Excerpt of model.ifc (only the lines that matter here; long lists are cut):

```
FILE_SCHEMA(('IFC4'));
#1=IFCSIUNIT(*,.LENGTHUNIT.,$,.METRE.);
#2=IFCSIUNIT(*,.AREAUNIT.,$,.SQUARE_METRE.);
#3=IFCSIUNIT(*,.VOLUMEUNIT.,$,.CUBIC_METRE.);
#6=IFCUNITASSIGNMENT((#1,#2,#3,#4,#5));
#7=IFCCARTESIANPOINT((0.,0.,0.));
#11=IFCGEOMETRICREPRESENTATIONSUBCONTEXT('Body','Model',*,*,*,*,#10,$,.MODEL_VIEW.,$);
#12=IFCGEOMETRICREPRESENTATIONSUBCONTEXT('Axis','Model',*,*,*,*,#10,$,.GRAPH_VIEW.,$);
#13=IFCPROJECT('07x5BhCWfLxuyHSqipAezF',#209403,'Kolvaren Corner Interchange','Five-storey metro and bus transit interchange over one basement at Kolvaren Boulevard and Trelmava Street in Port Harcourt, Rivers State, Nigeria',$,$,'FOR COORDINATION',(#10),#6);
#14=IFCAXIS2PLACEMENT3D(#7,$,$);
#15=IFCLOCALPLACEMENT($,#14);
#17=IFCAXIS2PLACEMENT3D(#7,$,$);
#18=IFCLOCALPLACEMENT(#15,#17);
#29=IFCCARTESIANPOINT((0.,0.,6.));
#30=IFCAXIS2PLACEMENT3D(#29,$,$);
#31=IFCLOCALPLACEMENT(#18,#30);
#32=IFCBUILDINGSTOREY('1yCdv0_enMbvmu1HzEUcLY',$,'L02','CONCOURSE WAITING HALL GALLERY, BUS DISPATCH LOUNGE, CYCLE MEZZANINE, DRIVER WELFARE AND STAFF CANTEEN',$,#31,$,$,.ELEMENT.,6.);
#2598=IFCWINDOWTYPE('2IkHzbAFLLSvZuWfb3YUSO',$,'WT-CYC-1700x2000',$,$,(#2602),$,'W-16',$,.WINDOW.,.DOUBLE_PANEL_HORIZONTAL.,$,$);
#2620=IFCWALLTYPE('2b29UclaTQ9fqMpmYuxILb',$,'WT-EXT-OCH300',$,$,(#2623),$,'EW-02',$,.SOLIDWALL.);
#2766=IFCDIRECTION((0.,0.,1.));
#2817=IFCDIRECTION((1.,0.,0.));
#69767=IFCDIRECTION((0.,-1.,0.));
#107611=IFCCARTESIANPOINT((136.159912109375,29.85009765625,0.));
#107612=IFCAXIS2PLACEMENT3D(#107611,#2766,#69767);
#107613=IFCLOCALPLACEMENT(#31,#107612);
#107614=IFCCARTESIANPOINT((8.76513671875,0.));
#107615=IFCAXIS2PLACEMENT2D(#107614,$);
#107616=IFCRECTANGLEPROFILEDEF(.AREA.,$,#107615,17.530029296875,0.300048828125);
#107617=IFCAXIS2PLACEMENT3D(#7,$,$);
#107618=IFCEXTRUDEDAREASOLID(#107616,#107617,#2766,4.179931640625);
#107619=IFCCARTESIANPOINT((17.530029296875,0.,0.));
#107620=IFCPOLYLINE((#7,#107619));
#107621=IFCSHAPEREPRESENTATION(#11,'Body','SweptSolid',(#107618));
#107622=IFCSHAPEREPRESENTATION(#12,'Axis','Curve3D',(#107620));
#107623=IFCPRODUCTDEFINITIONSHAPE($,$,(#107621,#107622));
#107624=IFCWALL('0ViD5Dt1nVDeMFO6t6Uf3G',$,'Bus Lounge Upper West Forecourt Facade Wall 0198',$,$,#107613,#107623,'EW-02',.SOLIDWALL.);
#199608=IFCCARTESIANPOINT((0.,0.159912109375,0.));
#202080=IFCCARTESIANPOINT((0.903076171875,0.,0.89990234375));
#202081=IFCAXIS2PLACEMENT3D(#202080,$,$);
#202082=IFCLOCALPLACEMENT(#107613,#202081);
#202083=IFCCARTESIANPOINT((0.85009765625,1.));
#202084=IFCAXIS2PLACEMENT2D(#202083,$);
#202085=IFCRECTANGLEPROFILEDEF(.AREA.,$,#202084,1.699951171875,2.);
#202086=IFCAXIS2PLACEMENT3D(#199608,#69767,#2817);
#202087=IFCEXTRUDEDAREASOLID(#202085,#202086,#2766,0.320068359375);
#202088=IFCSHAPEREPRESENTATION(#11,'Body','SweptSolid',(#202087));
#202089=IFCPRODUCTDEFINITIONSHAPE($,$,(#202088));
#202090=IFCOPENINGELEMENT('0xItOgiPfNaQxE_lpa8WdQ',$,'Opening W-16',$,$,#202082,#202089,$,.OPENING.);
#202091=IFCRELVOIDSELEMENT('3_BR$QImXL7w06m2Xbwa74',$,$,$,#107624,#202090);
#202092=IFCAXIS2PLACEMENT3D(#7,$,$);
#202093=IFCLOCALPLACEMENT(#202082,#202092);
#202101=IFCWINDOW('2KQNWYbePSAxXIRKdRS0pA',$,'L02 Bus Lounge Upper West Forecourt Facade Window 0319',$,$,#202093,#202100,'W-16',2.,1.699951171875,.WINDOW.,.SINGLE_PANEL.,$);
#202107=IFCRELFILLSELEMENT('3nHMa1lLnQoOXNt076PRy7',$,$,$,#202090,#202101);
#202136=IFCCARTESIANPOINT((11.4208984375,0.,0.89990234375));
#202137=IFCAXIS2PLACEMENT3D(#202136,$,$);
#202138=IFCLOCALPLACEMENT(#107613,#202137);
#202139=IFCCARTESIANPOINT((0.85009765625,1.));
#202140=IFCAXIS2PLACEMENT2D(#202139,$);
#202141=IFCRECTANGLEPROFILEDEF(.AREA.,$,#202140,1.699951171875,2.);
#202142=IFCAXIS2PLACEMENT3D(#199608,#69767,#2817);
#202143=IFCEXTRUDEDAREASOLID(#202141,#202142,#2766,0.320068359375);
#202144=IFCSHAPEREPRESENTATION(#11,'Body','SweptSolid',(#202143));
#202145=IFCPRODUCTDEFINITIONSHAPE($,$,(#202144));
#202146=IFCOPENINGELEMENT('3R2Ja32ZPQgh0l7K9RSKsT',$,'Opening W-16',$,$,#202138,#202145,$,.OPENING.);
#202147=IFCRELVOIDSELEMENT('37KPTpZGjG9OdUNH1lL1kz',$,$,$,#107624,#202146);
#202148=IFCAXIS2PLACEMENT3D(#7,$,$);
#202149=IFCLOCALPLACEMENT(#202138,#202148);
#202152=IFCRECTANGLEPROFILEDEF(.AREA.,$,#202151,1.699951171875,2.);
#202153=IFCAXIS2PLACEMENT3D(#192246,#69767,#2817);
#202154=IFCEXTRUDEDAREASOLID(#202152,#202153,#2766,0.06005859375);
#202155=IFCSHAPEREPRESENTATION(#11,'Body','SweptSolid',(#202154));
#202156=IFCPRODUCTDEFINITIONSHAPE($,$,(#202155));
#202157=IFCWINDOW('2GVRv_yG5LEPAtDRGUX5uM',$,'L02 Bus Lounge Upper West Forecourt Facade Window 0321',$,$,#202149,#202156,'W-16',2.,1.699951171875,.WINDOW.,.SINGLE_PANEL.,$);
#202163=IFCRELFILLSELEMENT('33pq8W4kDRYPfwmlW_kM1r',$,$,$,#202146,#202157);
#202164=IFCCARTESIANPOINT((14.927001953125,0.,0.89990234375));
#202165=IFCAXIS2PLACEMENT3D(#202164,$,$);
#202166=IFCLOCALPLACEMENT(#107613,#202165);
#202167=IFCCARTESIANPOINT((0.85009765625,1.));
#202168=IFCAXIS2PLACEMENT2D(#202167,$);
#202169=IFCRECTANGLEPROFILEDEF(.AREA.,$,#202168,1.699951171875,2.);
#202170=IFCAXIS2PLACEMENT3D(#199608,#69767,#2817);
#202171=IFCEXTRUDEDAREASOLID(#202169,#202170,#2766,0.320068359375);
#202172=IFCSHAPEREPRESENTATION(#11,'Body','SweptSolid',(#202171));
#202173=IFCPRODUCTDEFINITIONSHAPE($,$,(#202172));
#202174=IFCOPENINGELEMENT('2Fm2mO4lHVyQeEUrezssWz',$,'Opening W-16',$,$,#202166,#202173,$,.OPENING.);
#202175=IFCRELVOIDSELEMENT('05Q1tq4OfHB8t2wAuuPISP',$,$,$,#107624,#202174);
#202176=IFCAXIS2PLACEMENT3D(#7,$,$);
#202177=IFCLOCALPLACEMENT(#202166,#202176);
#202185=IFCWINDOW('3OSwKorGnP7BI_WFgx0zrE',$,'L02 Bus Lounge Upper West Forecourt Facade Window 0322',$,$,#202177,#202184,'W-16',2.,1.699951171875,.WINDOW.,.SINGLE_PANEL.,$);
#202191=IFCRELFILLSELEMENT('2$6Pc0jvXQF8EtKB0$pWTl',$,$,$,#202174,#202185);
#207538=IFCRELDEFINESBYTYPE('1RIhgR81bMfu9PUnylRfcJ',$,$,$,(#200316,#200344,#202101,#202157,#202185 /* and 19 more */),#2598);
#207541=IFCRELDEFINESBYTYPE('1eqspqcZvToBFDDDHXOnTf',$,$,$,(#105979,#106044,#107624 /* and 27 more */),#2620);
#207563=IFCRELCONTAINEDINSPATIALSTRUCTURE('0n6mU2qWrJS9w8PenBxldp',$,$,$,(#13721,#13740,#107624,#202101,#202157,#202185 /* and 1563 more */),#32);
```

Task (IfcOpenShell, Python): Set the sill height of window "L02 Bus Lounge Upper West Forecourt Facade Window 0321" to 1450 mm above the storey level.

```python
import numpy as np
import ifcopenshell
import ifcopenshell.api.geometry
import ifcopenshell.geom
import ifcopenshell.util.element
import ifcopenshell.util.placement
import ifcopenshell.util.shape
import ifcopenshell.util.unit

model = ifcopenshell.open("model.ifc")
unit_scale = ifcopenshell.util.unit.calculate_unit_scale(model)

window = model.by_guid("2GVRv_yG5LEPAtDRGUX5uM")
opening = window.FillsVoids[0].RelatingOpeningElement
storey = ifcopenshell.util.element.get_container(window, ifc_class="IfcBuildingStorey")
level = ifcopenshell.util.placement.get_local_placement(storey.ObjectPlacement)[2, 3]

# The opening's origin need not be at the sill, so measure its lowest point.
shape = ifcopenshell.geom.create_shape(ifcopenshell.geom.settings(), opening)
bottom = ifcopenshell.util.shape.get_shape_bottom_elevation(shape, shape.geometry) / unit_scale
dz = level + 1.45 / unit_scale - bottom

shift = np.array([0.0, 0.0, dz])
# The window is placed relative to its opening, so it follows when the opening moves.
matrix = ifcopenshell.util.placement.get_local_placement(opening.ObjectPlacement)
matrix[:3, 3] += shift
ifcopenshell.api.geometry.edit_object_placement(
    model, product=opening, matrix=matrix, is_si=False, should_transform_children=True
)

print(f"moved by {dz * unit_scale:+.3f} m")

model.write("model_updated.ifc")
```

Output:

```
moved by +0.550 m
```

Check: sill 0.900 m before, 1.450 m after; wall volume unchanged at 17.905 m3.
